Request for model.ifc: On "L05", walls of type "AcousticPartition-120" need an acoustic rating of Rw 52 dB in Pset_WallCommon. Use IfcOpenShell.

First a look at what the model holds.

```python
import ifcopenshell
import ifcopenshell.util.element

model = ifcopenshell.open("model.ifc")
print(model.schema)
storey = next(s for s in model.by_type("IfcBuildingStorey") if s.Name == "L05")
walls = [e for e in ifcopenshell.util.element.get_decomposition(storey) if e.is_a("IfcWall")]
seen = {}
for e in walls:
    element_type = ifcopenshell.util.element.get_type(e)
    key = (element_type.Name if element_type != e and element_type else None, ifcopenshell.util.element.get_pset(e, "Pset_WallCommon", "AcousticRating"))
    seen[key] = seen.get(key, 0) + 1
for (name, value), count in sorted(seen.items(), key=str):
    print(count, "x", name, "|", value)
```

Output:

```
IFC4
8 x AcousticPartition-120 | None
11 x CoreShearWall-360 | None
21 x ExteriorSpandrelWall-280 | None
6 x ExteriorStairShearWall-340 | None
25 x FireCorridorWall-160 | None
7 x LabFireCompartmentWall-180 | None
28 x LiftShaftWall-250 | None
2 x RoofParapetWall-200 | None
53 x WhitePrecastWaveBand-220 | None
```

```python
import ifcopenshell
import ifcopenshell.api.pset
import ifcopenshell.util.element

model = ifcopenshell.open("model.ifc")

storey = next(s for s in model.by_type("IfcBuildingStorey") if s.Name == "L05")
walls = [e for e in ifcopenshell.util.element.get_decomposition(storey) if e.is_a("IfcWall")]

count = 0
for e in walls:
    element_type = ifcopenshell.util.element.get_type(e)
    if element_type in (None, e) or element_type.Name != "AcousticPartition-120":
        continue
    # add_pset returns the element's existing set when there is one.
    pset = ifcopenshell.api.pset.add_pset(model, product=e, name="Pset_WallCommon")
    ifcopenshell.api.pset.edit_pset(model, pset=pset, properties={"AcousticRating": "Rw 52 dB"})
    count += 1

print(count, "walls updated")

model.write("model_edited.ifc")
```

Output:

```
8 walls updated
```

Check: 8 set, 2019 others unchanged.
